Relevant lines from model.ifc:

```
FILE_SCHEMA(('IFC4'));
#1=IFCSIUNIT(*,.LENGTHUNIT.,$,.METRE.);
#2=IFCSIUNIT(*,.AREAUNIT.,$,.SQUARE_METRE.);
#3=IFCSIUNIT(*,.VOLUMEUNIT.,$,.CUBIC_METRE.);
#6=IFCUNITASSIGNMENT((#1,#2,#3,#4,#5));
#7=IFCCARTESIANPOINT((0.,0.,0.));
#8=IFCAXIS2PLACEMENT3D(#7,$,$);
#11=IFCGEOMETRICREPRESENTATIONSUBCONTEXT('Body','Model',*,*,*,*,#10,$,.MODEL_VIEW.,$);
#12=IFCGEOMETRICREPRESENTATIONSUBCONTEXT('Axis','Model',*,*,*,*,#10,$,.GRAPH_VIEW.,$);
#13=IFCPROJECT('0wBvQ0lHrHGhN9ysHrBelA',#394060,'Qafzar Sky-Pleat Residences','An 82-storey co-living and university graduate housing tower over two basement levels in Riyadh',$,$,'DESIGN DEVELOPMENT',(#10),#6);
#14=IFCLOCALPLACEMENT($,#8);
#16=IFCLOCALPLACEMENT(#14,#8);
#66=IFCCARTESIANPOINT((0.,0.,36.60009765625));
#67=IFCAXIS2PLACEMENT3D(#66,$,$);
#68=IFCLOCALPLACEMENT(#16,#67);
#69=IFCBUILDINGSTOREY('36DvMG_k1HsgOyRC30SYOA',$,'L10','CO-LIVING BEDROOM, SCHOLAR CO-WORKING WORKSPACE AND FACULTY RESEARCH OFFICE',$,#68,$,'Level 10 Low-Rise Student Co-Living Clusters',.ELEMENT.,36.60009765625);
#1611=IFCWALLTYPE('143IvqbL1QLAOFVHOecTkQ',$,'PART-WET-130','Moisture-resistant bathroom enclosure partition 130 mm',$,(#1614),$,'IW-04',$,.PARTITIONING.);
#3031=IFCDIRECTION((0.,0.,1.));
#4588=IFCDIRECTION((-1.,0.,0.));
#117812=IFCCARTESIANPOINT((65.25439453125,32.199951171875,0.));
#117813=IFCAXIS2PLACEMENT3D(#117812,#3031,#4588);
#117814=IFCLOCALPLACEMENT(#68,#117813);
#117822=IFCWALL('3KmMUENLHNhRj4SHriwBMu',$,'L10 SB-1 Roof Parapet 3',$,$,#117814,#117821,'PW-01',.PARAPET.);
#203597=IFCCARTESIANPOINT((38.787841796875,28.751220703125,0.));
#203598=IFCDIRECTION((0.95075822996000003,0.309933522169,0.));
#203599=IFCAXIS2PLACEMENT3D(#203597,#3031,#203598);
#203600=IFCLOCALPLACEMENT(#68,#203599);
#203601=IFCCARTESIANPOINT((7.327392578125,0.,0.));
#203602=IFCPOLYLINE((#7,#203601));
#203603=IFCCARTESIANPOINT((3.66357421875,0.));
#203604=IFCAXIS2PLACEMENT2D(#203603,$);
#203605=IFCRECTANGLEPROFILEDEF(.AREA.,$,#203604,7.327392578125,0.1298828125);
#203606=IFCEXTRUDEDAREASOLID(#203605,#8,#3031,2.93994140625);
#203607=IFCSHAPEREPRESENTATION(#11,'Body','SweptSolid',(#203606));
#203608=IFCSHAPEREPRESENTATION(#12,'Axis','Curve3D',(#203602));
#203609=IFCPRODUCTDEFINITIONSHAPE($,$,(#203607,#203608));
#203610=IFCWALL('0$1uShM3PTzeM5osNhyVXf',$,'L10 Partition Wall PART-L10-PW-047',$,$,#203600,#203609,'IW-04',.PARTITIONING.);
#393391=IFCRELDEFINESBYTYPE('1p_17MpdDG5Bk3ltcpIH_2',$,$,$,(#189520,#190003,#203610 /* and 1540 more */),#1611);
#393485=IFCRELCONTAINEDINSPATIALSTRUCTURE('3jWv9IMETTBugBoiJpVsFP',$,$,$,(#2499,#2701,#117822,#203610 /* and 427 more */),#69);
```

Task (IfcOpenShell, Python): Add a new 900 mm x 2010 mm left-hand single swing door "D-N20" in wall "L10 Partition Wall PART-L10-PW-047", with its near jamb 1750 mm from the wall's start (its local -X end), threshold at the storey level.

```python
import numpy as np
import ifcopenshell
import ifcopenshell.api.feature
import ifcopenshell.api.geometry
import ifcopenshell.api.root
import ifcopenshell.api.spatial
import ifcopenshell.geom
import ifcopenshell.util.element
import ifcopenshell.util.placement
import ifcopenshell.util.representation
import ifcopenshell.util.shape
import ifcopenshell.util.unit

model = ifcopenshell.open("model.ifc")
unit_scale = ifcopenshell.util.unit.calculate_unit_scale(model)
settings = ifcopenshell.geom.settings()


def volume(element):
    """Net volume in cubic metres, openings subtracted."""
    shape = ifcopenshell.geom.create_shape(settings, element)
    return ifcopenshell.util.shape.get_volume(shape.geometry)


wall = model.by_guid("0$1uShM3PTzeM5osNhyVXf")
storey = ifcopenshell.util.element.get_container(wall, ifc_class="IfcBuildingStorey")
context = ifcopenshell.util.representation.get_context(model, "Model", "Body", "MODEL_VIEW")
before = volume(wall)

width, height, from_end, sill = 0.9, 2.01, 1.75, 0.0  # metres

# The wall runs along its own X axis, and the end named is its -X end.
wall_shape = ifcopenshell.geom.create_shape(settings, wall)
x, y, z = ifcopenshell.util.shape.get_vertices(wall_shape.geometry).T
start = x.min() + from_end
face, thickness = float(y.min()), float(y.max() - y.min())
wall_matrix = ifcopenshell.util.placement.get_local_placement(wall.ObjectPlacement)
level = ifcopenshell.util.placement.get_local_placement(storey.ObjectPlacement)[2, 3]


def in_wall(x, y):
    """Placement at x, y metres in the wall's axes, at sill height."""
    matrix = wall_matrix.copy()
    matrix[:, 3] = wall_matrix @ np.array([x / unit_scale, y / unit_scale, 0.0, 1.0])
    matrix[2, 3] = level + sill / unit_scale
    return matrix


# Opening: a box that overshoots both wall faces by 50 mm.
opening = ifcopenshell.api.root.create_entity(model, ifc_class="IfcOpeningElement", predefined_type="OPENING")
box = ifcopenshell.api.geometry.add_wall_representation(
    model, context=context, length=width, height=height, thickness=thickness + 0.1
)
ifcopenshell.api.geometry.assign_representation(model, product=opening, representation=box)
ifcopenshell.api.geometry.edit_object_placement(model, product=opening, matrix=in_wall(start, face - 0.05), is_si=False)
ifcopenshell.api.feature.add_feature(model, feature=opening, element=wall)

door = ifcopenshell.api.root.create_entity(model, ifc_class="IfcDoor", name="D-N20", predefined_type="DOOR")
door.OverallWidth, door.OverallHeight = width / unit_scale, height / unit_scale
door.OperationType = "SINGLE_SWING_LEFT"
body = ifcopenshell.api.geometry.add_door_representation(
    model,
    context=context,
    overall_width=door.OverallWidth,
    overall_height=door.OverallHeight,
    operation_type="SINGLE_SWING_LEFT",
    lining_properties={"LiningDepth": thickness / unit_scale, "ThresholdDepth": thickness / unit_scale},
)
ifcopenshell.api.geometry.assign_representation(model, product=door, representation=body)
ifcopenshell.api.spatial.assign_container(model, products=[door], relating_structure=storey)
ifcopenshell.api.feature.add_filling(model, opening=opening, element=door)

# The lining spans the wall, so the door starts at the wall face.
ifcopenshell.api.geometry.edit_object_placement(model, product=door, matrix=in_wall(start, face), is_si=False)

after = volume(wall)

print(f"wall volume {before:.3f} -> {after:.3f} m3")

model.write("model_v2.ifc")
```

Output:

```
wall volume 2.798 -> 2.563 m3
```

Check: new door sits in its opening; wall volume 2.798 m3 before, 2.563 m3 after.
